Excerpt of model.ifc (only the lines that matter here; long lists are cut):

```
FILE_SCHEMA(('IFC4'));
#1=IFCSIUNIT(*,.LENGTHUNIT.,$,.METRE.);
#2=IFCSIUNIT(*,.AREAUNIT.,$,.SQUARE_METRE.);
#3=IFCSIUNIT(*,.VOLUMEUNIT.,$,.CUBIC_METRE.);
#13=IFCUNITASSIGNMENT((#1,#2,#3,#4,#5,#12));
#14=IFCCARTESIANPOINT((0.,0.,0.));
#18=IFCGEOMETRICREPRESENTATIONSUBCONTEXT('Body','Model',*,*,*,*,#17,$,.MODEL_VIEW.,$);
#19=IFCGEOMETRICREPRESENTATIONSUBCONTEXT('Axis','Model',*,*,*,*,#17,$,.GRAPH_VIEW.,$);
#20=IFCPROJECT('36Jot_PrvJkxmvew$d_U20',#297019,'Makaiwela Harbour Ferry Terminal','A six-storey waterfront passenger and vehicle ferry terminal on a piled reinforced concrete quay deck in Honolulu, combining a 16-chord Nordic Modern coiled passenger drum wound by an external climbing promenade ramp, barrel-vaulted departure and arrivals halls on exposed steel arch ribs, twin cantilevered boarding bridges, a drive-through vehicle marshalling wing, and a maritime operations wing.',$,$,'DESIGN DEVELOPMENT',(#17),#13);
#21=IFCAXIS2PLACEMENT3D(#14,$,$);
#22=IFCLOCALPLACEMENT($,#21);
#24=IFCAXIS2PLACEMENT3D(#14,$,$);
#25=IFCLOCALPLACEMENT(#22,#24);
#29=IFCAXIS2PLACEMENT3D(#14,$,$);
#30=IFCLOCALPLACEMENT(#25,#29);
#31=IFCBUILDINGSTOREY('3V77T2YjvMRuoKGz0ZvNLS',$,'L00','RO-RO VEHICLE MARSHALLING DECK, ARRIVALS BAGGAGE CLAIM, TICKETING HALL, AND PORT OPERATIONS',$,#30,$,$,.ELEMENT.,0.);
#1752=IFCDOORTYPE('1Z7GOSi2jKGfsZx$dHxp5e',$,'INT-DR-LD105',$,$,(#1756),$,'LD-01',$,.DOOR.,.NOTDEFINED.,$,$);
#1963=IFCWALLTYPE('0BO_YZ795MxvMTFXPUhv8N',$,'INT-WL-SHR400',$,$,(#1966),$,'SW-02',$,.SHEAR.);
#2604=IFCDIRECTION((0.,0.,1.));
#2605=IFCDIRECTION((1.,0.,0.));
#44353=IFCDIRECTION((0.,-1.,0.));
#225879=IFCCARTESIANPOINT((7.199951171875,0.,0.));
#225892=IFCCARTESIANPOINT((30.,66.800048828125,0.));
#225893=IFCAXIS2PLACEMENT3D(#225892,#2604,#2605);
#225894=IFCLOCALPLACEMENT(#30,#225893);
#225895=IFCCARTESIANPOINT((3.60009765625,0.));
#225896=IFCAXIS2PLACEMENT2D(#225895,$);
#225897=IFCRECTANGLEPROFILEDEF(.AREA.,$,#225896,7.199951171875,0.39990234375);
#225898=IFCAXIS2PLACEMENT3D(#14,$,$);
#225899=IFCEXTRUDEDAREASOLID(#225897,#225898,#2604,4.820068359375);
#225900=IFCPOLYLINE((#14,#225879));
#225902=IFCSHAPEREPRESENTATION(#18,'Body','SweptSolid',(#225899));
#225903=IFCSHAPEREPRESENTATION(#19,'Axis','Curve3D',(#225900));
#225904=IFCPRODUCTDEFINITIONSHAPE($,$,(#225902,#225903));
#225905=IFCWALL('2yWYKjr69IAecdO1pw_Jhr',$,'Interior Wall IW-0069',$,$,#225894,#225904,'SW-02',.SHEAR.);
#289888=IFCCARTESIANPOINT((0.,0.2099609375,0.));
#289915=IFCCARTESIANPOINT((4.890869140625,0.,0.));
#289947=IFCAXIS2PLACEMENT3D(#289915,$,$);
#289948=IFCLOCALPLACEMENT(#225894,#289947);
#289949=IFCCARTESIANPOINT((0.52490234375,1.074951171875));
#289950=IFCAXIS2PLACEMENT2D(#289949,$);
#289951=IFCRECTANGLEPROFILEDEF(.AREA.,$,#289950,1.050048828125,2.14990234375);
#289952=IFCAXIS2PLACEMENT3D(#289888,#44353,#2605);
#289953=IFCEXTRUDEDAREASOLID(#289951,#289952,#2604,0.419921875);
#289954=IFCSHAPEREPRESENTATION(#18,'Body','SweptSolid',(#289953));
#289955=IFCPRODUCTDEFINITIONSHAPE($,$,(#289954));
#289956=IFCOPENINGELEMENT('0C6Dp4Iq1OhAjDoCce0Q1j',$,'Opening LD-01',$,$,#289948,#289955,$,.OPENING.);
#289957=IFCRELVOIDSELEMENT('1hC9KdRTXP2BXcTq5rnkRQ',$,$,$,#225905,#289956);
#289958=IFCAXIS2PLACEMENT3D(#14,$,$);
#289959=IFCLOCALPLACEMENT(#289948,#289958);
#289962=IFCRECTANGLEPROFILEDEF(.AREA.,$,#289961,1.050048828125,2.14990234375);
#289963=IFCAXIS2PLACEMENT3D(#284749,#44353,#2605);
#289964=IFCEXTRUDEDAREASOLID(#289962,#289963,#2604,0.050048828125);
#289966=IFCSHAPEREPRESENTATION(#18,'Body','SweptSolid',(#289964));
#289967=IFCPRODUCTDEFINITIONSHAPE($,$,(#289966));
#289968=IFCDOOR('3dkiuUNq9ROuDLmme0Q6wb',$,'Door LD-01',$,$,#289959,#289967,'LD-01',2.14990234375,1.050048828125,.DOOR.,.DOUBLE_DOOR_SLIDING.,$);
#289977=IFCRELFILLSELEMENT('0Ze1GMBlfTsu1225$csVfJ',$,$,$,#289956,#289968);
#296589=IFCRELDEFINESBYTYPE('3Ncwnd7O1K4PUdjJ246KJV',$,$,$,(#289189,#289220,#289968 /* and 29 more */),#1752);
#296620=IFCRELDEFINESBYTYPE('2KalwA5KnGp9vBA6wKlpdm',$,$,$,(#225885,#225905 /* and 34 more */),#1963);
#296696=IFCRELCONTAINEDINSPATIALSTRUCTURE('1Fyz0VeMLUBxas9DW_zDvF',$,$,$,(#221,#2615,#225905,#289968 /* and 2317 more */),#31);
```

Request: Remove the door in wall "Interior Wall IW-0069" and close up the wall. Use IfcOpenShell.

```python
import ifcopenshell
import ifcopenshell.api.feature
import ifcopenshell.api.root
import ifcopenshell.geom
import ifcopenshell.util.shape

model = ifcopenshell.open("model.ifc")
settings = ifcopenshell.geom.settings()


def volume(element):
    """Net volume in cubic metres, openings subtracted."""
    shape = ifcopenshell.geom.create_shape(settings, element)
    return ifcopenshell.util.shape.get_volume(shape.geometry)


door = model.by_id(289968)
opening = door.FillsVoids[0].RelatingOpeningElement
wall = opening.VoidsElements[0].RelatingBuildingElement
before = volume(wall)

ifcopenshell.api.root.remove_product(model, product=door)
ifcopenshell.api.feature.remove_feature(model, feature=opening)

after = volume(wall)

print(f"wall volume {before:.3f} -> {after:.3f} m3")

model.write("model-out.ifc")
```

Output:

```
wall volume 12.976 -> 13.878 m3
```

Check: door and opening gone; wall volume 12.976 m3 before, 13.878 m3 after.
